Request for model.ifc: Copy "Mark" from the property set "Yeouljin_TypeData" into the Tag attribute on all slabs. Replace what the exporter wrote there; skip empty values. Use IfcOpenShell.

First a look at what the model holds.

```python
import ifcopenshell
import ifcopenshell.util.element

model = ifcopenshell.open("model.ifc")
print(model.schema)
slabs = model.by_type("IfcSlab")
print(len(slabs), "slabs")
for e in slabs[:8]:
    source = ifcopenshell.util.element.get_pset(e, "Yeouljin_TypeData", "Mark")
    target = e.Tag
    print(e.id(), repr(source), repr(target), sep=" | ")
```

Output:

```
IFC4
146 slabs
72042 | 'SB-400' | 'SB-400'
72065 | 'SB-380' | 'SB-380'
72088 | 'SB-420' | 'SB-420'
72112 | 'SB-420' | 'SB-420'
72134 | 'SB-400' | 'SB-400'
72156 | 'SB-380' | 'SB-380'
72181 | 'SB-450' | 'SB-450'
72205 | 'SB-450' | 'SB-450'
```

```python
import ifcopenshell
import ifcopenshell.util.element

model = ifcopenshell.open("model.ifc")

count = 0
for e in model.by_type("IfcSlab"):
    value = ifcopenshell.util.element.get_pset(e, "Yeouljin_TypeData", "Mark")
    current = e.Tag
    if not value or not value.strip() or current == value:
        continue
    e.Tag = value
    count += 1

print(count, "slabs updated")

model.write("model_edited.ifc")
```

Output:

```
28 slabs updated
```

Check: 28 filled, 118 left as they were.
